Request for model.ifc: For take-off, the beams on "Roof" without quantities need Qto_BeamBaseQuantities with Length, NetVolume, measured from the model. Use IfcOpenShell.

First a look at what the model holds.

```python
import ifcopenshell
import ifcopenshell.util.element
import ifcopenshell.util.unit

model = ifcopenshell.open("model.ifc")
print(model.schema)
for unit_type in ("LENGTHUNIT", "AREAUNIT", "VOLUMEUNIT"):
    print(unit_type, ifcopenshell.util.unit.calculate_unit_scale(model, unit_type))
storey = next(s for s in model.by_type("IfcBuildingStorey") if s.Name == "Roof")
beams = [e for e in ifcopenshell.util.element.get_decomposition(storey) if e.is_a("IfcBeam")]
for e in sorted(beams, key=lambda e: e.id()):
    print(e.id(), e.is_a(), e.Name, list(ifcopenshell.util.element.get_psets(e, qtos_only=True)), sep=" | ")
```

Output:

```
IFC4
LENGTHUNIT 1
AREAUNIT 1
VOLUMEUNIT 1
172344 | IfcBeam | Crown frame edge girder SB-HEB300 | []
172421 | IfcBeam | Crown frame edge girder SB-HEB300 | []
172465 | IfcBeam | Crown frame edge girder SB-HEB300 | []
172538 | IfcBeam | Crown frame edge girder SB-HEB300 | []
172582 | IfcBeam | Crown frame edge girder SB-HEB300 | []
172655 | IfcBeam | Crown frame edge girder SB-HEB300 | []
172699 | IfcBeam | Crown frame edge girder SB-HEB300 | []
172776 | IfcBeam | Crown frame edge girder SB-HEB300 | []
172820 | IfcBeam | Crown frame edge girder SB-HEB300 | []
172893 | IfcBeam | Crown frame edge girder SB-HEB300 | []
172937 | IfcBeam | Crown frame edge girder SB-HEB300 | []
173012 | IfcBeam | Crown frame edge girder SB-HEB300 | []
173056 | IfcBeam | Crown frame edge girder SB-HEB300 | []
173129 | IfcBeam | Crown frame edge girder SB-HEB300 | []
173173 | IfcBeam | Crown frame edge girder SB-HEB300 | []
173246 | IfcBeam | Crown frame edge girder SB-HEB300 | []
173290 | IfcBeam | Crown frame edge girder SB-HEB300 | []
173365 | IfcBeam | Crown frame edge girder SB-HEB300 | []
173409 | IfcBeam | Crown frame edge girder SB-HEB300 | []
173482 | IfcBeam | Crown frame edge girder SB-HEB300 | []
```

```python
import ifcopenshell
import ifcopenshell.api.pset
import ifcopenshell.geom
import ifcopenshell.util.element
import ifcopenshell.util.shape
import ifcopenshell.util.unit

model = ifcopenshell.open("model.ifc")
unit_scale = ifcopenshell.util.unit.calculate_unit_scale(model)
volume_scale = ifcopenshell.util.unit.calculate_unit_scale(model, "VOLUMEUNIT")
settings = ifcopenshell.geom.settings()

storey = next(s for s in model.by_type("IfcBuildingStorey") if s.Name == "Roof")
beams = [e for e in ifcopenshell.util.element.get_decomposition(storey) if e.is_a("IfcBeam")]

for e in sorted(beams, key=lambda e: e.id()):
    if ifcopenshell.util.element.get_psets(e, qtos_only=True, should_inherit=False):
        continue
    # Geometry comes back in metres, in the element's own axes.
    shape = ifcopenshell.geom.create_shape(settings, e)
    values = {
        "Length": ifcopenshell.util.shape.get_max_xyz(shape.geometry) / unit_scale,
        "NetVolume": ifcopenshell.util.shape.get_volume(shape.geometry) / volume_scale,
    }
    qto = ifcopenshell.api.pset.add_qto(model, product=e, name="Qto_BeamBaseQuantities")
    ifcopenshell.api.pset.edit_qto(model, qto=qto, properties=values)
    print(e.id(), {k: round(v, 3) for k, v in values.items()})

model.write("model_edited.ifc")
```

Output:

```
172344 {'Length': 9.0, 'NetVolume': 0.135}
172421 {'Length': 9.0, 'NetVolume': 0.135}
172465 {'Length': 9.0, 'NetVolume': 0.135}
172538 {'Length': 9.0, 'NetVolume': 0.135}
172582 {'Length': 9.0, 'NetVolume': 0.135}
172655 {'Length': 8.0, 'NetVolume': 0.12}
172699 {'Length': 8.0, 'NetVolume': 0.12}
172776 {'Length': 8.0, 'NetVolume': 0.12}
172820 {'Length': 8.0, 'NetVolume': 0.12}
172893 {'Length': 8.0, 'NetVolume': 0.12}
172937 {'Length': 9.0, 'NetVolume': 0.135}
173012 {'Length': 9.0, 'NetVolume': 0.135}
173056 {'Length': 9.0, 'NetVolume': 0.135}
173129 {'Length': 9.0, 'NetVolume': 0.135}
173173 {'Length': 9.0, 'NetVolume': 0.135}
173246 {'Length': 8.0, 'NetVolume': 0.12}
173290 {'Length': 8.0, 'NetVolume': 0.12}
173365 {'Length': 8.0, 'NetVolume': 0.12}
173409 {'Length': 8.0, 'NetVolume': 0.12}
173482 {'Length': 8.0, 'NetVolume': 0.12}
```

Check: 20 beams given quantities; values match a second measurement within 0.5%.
